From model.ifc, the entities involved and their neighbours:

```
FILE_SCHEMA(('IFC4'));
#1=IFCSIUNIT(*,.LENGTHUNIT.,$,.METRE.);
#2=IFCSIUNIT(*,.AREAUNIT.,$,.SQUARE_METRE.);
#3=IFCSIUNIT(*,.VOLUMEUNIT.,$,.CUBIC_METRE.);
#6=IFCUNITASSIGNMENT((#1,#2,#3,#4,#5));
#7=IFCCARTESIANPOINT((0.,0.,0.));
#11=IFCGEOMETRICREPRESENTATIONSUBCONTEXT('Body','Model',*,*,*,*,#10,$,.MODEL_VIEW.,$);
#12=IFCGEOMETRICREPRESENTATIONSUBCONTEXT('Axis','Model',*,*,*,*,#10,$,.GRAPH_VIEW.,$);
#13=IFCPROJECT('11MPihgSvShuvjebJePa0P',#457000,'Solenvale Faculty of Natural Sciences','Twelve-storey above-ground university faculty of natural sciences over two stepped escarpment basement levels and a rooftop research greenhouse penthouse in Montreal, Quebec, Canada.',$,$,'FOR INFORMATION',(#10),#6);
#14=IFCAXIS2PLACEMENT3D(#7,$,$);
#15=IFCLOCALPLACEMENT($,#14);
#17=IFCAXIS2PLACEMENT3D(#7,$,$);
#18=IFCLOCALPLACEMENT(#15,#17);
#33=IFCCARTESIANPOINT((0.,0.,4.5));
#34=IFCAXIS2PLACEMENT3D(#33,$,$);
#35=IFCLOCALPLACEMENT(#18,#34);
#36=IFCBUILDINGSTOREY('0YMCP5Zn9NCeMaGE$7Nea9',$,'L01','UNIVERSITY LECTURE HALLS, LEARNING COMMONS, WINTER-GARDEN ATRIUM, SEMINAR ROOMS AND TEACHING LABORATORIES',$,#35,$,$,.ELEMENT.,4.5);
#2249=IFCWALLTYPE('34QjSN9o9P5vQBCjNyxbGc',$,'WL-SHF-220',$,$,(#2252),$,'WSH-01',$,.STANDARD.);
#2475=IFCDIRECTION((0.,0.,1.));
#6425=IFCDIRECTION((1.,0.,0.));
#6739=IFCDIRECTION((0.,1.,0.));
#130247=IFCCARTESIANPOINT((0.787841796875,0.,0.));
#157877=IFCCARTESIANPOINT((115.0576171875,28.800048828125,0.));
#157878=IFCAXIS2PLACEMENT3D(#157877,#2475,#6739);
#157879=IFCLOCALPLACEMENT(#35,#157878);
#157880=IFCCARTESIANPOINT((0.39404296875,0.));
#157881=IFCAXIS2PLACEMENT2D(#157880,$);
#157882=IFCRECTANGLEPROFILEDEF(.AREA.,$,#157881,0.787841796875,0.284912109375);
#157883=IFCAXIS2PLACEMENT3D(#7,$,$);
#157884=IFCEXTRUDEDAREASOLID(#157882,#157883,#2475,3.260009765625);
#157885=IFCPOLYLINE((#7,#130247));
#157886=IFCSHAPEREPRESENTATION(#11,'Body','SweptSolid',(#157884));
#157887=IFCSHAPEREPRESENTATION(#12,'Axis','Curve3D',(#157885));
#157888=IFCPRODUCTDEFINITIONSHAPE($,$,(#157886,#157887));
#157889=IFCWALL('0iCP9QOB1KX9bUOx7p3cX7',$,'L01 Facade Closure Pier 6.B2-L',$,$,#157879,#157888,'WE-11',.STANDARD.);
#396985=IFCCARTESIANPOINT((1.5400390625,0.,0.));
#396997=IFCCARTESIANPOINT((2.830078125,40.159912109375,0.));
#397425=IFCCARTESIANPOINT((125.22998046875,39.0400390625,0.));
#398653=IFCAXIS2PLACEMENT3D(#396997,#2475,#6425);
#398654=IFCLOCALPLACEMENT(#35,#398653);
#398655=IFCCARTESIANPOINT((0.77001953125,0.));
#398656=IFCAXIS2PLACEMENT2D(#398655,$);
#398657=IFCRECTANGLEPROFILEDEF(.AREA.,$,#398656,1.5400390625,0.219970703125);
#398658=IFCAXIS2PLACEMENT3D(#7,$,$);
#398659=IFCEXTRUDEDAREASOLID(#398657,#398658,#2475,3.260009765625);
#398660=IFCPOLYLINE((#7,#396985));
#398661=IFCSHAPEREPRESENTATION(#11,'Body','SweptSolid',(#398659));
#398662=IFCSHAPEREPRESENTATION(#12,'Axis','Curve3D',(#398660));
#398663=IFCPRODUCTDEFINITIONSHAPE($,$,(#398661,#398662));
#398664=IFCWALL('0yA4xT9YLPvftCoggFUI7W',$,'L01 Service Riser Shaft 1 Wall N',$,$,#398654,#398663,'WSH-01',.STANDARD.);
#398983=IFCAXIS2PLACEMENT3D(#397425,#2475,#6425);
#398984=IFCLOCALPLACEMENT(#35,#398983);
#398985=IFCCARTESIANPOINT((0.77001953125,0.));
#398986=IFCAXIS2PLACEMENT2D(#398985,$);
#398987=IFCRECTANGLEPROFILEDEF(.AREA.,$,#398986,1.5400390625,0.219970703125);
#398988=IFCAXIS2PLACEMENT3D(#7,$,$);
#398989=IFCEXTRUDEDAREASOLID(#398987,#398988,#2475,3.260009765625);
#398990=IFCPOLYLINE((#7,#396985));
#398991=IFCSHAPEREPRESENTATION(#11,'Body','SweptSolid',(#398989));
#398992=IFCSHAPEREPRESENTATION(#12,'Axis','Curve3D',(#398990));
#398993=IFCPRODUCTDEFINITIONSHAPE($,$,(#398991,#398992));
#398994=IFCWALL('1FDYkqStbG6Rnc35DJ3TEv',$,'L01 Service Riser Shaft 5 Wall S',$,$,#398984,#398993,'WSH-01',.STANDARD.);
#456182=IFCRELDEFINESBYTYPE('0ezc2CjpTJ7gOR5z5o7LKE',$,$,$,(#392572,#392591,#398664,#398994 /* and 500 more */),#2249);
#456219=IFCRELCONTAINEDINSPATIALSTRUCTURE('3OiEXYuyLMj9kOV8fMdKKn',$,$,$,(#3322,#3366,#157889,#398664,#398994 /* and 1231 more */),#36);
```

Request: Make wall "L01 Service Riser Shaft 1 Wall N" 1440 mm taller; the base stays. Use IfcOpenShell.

```python
import ifcopenshell
import ifcopenshell.geom
import ifcopenshell.util.representation
import ifcopenshell.util.shape
import ifcopenshell.util.unit

model = ifcopenshell.open("model.ifc")
unit_scale = ifcopenshell.util.unit.calculate_unit_scale(model)
settings = ifcopenshell.geom.settings()


def volume(element):
    """Net volume in cubic metres, openings subtracted."""
    shape = ifcopenshell.geom.create_shape(settings, element)
    return ifcopenshell.util.shape.get_volume(shape.geometry)


wall = model.by_id(398664)
before = volume(wall)

body = ifcopenshell.util.representation.get_representation(wall, "Model", "Body")
solid = body.Items[0]
old_height = solid.Depth
solid.Depth += 1.44 / unit_scale
after = volume(wall)

print(f"height {old_height:g} -> {solid.Depth:g}, volume {before:.3f} -> {after:.3f} m3")

model.write("model_v2.ifc")
```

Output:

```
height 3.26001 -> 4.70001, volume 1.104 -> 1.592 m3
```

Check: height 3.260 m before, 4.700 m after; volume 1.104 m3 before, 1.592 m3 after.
